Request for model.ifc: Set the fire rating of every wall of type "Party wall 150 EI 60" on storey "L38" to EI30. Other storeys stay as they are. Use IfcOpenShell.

First a look at what the model holds.

```python
import ifcopenshell
import ifcopenshell.util.element

model = ifcopenshell.open("model.ifc")
print(model.schema)
storey = next(s for s in model.by_type("IfcBuildingStorey") if s.Name == "L38")
walls = [e for e in ifcopenshell.util.element.get_decomposition(storey) if e.is_a("IfcWall")]
seen = {}
for e in walls:
    element_type = ifcopenshell.util.element.get_type(e)
    key = (element_type.Name if element_type != e and element_type else None, ifcopenshell.util.element.get_pset(e, "Pset_WallCommon", "FireRating"))
    seen[key] = seen.get(key, 0) + 1
for (name, value), count in sorted(seen.items(), key=str):
    print(count, "x", name, "|", value)
```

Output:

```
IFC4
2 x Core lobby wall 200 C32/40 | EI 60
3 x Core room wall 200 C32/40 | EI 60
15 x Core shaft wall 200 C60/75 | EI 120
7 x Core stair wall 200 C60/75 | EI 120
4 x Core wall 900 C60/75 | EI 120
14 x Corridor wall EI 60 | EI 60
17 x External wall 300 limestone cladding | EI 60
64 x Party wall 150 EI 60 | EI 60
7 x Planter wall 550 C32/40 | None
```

```python
import ifcopenshell
import ifcopenshell.api.pset
import ifcopenshell.util.element

model = ifcopenshell.open("model.ifc")

storey = next(s for s in model.by_type("IfcBuildingStorey") if s.Name == "L38")
walls = [e for e in ifcopenshell.util.element.get_decomposition(storey) if e.is_a("IfcWall")]

count = 0
for e in walls:
    element_type = ifcopenshell.util.element.get_type(e)
    if element_type in (None, e) or element_type.Name != "Party wall 150 EI 60":
        continue
    found = ifcopenshell.util.element.get_pset(e, "Pset_WallCommon", should_inherit=False)
    if found:
        pset = model.by_id(found["id"])
        if len(ifcopenshell.util.element.get_elements_by_pset(pset)) > 1:
            pset = ifcopenshell.api.pset.unshare_pset(model, products=[e], pset=pset)[0]
    else:
        pset = ifcopenshell.api.pset.add_pset(model, product=e, name="Pset_WallCommon")
    ifcopenshell.api.pset.edit_pset(model, pset=pset, properties={"FireRating": "EI30"})
    count += 1

print(count, "walls updated")

model.write("model-out.ifc")
```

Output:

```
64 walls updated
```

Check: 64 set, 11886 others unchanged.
